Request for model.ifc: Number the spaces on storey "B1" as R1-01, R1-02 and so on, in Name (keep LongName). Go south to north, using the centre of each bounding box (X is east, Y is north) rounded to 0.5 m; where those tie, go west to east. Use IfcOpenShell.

First a look at what the model holds.

```python
import ifcopenshell
import ifcopenshell.util.element
import ifcopenshell.util.placement

model = ifcopenshell.open("model.ifc")
print(model.schema)
storey = next(s for s in model.by_type("IfcBuildingStorey") if s.Name == "B1")
spaces = [e for e in ifcopenshell.util.element.get_decomposition(storey) if e.is_a("IfcSpace")]
for e in sorted(spaces, key=lambda e: e.id()):
    origin = ifcopenshell.util.placement.get_local_placement(e.ObjectPlacement)[:3, 3]
    print(e.id(), e.Name, e.LongName, origin.round(2) + 0.0, sep=" | ")
```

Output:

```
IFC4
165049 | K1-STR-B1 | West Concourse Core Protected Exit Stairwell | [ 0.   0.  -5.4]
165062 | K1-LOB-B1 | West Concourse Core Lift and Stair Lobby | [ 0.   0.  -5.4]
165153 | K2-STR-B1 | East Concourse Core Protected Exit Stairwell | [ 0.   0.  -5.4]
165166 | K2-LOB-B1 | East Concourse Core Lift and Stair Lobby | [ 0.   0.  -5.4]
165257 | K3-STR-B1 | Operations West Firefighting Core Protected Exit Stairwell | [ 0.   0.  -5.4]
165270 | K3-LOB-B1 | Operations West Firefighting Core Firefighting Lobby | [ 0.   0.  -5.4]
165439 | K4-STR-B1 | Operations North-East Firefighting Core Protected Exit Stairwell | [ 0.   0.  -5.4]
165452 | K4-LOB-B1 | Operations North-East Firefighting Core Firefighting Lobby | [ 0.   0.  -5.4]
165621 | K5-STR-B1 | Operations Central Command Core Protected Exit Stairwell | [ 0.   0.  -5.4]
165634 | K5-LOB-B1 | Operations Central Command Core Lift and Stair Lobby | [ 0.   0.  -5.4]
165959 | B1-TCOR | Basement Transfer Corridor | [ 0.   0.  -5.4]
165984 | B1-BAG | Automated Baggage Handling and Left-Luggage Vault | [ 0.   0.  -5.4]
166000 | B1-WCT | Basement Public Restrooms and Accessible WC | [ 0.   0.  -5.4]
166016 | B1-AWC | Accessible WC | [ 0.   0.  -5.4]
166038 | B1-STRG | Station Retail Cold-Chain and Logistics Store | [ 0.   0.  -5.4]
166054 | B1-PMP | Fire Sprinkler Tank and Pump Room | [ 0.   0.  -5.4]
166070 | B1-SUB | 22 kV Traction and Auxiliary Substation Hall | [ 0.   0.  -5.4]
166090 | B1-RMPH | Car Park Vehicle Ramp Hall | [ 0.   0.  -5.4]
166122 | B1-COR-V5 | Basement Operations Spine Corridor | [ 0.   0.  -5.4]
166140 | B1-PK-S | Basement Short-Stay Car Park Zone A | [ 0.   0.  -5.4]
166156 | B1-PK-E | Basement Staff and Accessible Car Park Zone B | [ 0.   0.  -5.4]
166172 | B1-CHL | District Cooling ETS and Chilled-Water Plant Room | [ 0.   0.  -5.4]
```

```python
import ifcopenshell
import ifcopenshell.geom
import ifcopenshell.util.element
import ifcopenshell.util.shape

model = ifcopenshell.open("model.ifc")
settings = ifcopenshell.geom.settings()
settings.set("use-world-coords", True)


def centre(element):
    shape = ifcopenshell.geom.create_shape(settings, element)
    return ifcopenshell.util.shape.get_bbox_centroid(shape.geometry)


storey = next(s for s in model.by_type("IfcBuildingStorey") if s.Name == "B1")
spaces = [e for e in ifcopenshell.util.element.get_decomposition(storey) if e.is_a("IfcSpace")]

# Insertion points can sit at a corner or the storey origin, so sort by the geometry (in metres).
centres = {e: centre(e) for e in spaces}
spaces.sort(key=lambda e: (round(centres[e][1] / 0.5), centres[e][0]))

for i, e in enumerate(spaces, start=1):
    number = f"R1-{i:02d}"
    e.Name = number
    print(e.id(), number)

model.write("model_edited.ifc")
```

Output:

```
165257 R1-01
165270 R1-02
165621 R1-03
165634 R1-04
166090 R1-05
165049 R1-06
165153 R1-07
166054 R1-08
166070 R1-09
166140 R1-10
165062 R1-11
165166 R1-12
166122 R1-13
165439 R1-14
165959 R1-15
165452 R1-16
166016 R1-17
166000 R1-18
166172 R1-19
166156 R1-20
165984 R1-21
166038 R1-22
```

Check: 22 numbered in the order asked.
